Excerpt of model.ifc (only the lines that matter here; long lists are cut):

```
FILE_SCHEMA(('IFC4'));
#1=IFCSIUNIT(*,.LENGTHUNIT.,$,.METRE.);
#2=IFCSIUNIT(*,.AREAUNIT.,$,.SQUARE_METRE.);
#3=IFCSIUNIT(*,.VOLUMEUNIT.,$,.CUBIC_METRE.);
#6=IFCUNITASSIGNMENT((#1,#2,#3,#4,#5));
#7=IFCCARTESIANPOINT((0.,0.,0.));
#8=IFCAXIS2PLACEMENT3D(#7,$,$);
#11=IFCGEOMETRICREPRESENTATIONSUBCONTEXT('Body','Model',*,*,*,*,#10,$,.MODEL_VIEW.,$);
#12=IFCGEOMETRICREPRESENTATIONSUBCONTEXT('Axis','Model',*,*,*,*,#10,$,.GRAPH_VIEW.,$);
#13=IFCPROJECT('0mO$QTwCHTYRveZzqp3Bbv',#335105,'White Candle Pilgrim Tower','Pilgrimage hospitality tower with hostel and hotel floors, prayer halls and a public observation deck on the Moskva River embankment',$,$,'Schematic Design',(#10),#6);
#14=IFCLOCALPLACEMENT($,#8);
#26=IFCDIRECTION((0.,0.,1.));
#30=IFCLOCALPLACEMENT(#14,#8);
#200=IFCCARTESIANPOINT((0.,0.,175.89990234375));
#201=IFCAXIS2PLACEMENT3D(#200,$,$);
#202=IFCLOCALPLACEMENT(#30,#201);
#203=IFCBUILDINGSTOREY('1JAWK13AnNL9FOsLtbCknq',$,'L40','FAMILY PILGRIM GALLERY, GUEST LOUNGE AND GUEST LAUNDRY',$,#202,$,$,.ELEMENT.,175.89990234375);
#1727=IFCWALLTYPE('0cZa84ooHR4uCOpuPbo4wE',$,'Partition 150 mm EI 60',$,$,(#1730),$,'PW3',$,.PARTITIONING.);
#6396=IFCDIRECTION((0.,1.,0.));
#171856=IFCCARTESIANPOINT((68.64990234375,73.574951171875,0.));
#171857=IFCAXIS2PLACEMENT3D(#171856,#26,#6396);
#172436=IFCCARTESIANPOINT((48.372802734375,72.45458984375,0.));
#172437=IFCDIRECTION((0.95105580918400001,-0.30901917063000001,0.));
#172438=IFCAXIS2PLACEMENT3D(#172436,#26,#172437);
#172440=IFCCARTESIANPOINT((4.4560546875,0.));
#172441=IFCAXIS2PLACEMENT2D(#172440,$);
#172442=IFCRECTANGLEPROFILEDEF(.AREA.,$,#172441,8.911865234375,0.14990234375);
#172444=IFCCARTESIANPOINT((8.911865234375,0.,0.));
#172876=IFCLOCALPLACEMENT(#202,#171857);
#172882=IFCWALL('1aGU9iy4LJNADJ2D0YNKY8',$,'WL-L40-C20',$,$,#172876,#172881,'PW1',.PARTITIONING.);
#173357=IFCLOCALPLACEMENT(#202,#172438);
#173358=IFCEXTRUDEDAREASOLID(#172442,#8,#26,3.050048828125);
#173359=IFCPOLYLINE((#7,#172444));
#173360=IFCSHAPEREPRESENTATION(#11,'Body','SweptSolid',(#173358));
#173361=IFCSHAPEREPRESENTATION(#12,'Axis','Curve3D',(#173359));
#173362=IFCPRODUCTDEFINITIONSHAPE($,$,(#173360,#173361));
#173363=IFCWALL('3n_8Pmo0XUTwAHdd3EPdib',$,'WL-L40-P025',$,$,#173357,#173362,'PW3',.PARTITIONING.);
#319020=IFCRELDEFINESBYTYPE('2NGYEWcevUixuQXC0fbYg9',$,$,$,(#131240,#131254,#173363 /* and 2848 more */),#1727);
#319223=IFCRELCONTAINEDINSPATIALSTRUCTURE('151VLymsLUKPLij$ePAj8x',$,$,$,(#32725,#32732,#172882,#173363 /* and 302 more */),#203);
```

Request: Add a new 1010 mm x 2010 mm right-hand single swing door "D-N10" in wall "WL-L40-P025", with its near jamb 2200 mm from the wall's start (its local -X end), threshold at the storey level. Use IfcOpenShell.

```python
import numpy as np
import ifcopenshell
import ifcopenshell.api.feature
import ifcopenshell.api.geometry
import ifcopenshell.api.root
import ifcopenshell.api.spatial
import ifcopenshell.geom
import ifcopenshell.util.element
import ifcopenshell.util.placement
import ifcopenshell.util.representation
import ifcopenshell.util.shape
import ifcopenshell.util.unit

model = ifcopenshell.open("model.ifc")
unit_scale = ifcopenshell.util.unit.calculate_unit_scale(model)
settings = ifcopenshell.geom.settings()


def volume(element):
    """Net volume in cubic metres, openings subtracted."""
    shape = ifcopenshell.geom.create_shape(settings, element)
    return ifcopenshell.util.shape.get_volume(shape.geometry)


wall = model.by_guid("3n_8Pmo0XUTwAHdd3EPdib")
storey = ifcopenshell.util.element.get_container(wall, ifc_class="IfcBuildingStorey")
context = ifcopenshell.util.representation.get_context(model, "Model", "Body", "MODEL_VIEW")
before = volume(wall)

width, height, from_end, sill = 1.01, 2.01, 2.2, 0.0  # metres

# The wall runs along its own X axis, and the end named is its -X end.
wall_shape = ifcopenshell.geom.create_shape(settings, wall)
x, y, z = ifcopenshell.util.shape.get_vertices(wall_shape.geometry).T
start = x.min() + from_end
face, thickness = float(y.min()), float(y.max() - y.min())
wall_matrix = ifcopenshell.util.placement.get_local_placement(wall.ObjectPlacement)
level = ifcopenshell.util.placement.get_local_placement(storey.ObjectPlacement)[2, 3]


def in_wall(x, y):
    """Placement at x, y metres in the wall's axes, at sill height."""
    matrix = wall_matrix.copy()
    matrix[:, 3] = wall_matrix @ np.array([x / unit_scale, y / unit_scale, 0.0, 1.0])
    matrix[2, 3] = level + sill / unit_scale
    return matrix


# Opening: a box that overshoots both wall faces by 50 mm.
opening = ifcopenshell.api.root.create_entity(model, ifc_class="IfcOpeningElement", predefined_type="OPENING")
box = ifcopenshell.api.geometry.add_wall_representation(
    model, context=context, length=width, height=height, thickness=thickness + 0.1
)
ifcopenshell.api.geometry.assign_representation(model, product=opening, representation=box)
ifcopenshell.api.geometry.edit_object_placement(model, product=opening, matrix=in_wall(start, face - 0.05), is_si=False)
ifcopenshell.api.feature.add_feature(model, feature=opening, element=wall)

door = ifcopenshell.api.root.create_entity(model, ifc_class="IfcDoor", name="D-N10", predefined_type="DOOR")
door.OverallWidth, door.OverallHeight = width / unit_scale, height / unit_scale
door.OperationType = "SINGLE_SWING_RIGHT"
body = ifcopenshell.api.geometry.add_door_representation(
    model,
    context=context,
    overall_width=door.OverallWidth,
    overall_height=door.OverallHeight,
    operation_type="SINGLE_SWING_RIGHT",
    lining_properties={"LiningDepth": thickness / unit_scale, "ThresholdDepth": thickness / unit_scale},
)
ifcopenshell.api.geometry.assign_representation(model, product=door, representation=body)
ifcopenshell.api.spatial.assign_container(model, products=[door], relating_structure=storey)
ifcopenshell.api.feature.add_filling(model, opening=opening, element=door)

# The lining spans the wall, so the door starts at the wall face.
ifcopenshell.api.geometry.edit_object_placement(model, product=door, matrix=in_wall(start, face), is_si=False)

after = volume(wall)

print(f"wall volume {before:.3f} -> {after:.3f} m3")

model.write("model_edited.ifc")
```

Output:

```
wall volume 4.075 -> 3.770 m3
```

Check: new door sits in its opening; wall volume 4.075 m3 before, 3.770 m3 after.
